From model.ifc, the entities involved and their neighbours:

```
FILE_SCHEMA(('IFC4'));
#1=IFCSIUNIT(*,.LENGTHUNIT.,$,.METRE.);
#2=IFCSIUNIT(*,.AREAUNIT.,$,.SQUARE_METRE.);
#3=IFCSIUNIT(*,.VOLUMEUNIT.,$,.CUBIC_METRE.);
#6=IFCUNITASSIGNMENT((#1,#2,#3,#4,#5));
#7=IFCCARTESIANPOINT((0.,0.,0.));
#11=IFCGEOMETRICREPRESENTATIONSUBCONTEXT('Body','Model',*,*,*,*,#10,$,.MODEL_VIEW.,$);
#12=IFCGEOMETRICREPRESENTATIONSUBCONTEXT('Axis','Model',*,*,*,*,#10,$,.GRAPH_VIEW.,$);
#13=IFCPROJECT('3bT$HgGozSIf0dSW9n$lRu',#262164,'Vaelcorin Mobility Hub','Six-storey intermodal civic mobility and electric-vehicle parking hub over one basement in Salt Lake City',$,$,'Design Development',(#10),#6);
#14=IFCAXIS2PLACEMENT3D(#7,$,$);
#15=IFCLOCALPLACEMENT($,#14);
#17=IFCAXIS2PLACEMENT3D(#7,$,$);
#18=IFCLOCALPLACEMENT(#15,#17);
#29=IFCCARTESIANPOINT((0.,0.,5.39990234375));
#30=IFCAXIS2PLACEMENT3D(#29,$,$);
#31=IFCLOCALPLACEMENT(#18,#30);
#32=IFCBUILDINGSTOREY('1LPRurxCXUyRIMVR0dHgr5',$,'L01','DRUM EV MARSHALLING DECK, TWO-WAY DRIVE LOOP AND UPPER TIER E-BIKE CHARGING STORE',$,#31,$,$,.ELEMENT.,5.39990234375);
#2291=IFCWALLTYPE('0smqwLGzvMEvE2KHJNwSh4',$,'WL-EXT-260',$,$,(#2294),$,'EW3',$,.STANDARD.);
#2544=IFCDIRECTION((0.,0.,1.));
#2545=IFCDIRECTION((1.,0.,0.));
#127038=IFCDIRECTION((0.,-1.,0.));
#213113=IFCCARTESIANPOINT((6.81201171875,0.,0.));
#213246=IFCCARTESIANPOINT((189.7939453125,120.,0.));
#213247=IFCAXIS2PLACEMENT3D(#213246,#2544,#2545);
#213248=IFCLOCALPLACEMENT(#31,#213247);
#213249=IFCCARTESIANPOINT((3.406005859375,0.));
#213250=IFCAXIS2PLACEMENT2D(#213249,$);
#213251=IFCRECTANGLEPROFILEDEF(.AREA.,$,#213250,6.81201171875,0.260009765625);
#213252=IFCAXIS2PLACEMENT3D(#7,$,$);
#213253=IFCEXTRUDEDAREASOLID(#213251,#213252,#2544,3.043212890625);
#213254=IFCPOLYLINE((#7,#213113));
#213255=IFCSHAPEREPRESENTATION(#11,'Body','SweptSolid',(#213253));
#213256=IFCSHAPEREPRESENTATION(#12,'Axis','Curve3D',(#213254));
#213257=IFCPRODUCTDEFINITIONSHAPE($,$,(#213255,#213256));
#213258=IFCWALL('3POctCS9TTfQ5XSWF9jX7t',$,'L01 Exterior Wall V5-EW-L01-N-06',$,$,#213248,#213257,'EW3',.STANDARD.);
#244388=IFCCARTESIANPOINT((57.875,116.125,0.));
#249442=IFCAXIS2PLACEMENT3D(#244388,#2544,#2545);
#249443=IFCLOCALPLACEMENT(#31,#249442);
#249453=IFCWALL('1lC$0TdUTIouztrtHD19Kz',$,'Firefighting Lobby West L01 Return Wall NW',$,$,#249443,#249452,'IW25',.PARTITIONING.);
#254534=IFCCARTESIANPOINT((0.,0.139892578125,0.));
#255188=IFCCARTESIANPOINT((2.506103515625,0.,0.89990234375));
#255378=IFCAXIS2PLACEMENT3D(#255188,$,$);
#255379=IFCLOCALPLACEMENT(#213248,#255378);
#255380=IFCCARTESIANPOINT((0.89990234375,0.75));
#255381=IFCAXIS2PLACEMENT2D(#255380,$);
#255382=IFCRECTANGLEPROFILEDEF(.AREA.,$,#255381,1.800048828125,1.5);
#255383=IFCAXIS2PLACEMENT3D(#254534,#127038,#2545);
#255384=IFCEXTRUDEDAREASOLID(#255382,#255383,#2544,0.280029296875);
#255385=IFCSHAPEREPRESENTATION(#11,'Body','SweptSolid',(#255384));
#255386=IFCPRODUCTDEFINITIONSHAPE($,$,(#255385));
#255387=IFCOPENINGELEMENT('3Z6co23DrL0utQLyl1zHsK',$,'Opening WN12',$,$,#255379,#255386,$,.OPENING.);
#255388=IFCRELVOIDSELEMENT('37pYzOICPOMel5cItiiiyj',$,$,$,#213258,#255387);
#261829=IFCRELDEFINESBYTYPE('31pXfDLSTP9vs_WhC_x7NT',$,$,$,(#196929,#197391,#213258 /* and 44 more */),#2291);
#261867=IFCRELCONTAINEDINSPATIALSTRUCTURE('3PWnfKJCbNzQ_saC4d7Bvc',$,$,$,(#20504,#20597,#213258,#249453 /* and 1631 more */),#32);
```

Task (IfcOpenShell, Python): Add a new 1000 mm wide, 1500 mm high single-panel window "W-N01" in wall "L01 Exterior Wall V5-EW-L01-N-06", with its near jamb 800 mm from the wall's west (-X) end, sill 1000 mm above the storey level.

```python
import numpy as np
import ifcopenshell
import ifcopenshell.api.feature
import ifcopenshell.api.geometry
import ifcopenshell.api.root
import ifcopenshell.api.spatial
import ifcopenshell.geom
import ifcopenshell.util.element
import ifcopenshell.util.placement
import ifcopenshell.util.representation
import ifcopenshell.util.shape
import ifcopenshell.util.unit

model = ifcopenshell.open("model.ifc")
unit_scale = ifcopenshell.util.unit.calculate_unit_scale(model)
settings = ifcopenshell.geom.settings()


def volume(element):
    """Net volume in cubic metres, openings subtracted."""
    shape = ifcopenshell.geom.create_shape(settings, element)
    return ifcopenshell.util.shape.get_volume(shape.geometry)


wall = model.by_guid("3POctCS9TTfQ5XSWF9jX7t")
storey = ifcopenshell.util.element.get_container(wall, ifc_class="IfcBuildingStorey")
context = ifcopenshell.util.representation.get_context(model, "Model", "Body", "MODEL_VIEW")
before = volume(wall)

width, height, from_end, sill = 1, 1.5, 0.8, 1  # metres

# The wall runs along its own X axis, and the end named is its -X end.
wall_shape = ifcopenshell.geom.create_shape(settings, wall)
x, y, z = ifcopenshell.util.shape.get_vertices(wall_shape.geometry).T
start = x.min() + from_end
face, thickness = float(y.min()), float(y.max() - y.min())
wall_matrix = ifcopenshell.util.placement.get_local_placement(wall.ObjectPlacement)
level = ifcopenshell.util.placement.get_local_placement(storey.ObjectPlacement)[2, 3]


def in_wall(x, y):
    """Placement at x, y metres in the wall's axes, at sill height."""
    matrix = wall_matrix.copy()
    matrix[:, 3] = wall_matrix @ np.array([x / unit_scale, y / unit_scale, 0.0, 1.0])
    matrix[2, 3] = level + sill / unit_scale
    return matrix


# Opening: a box that overshoots both wall faces by 50 mm.
opening = ifcopenshell.api.root.create_entity(model, ifc_class="IfcOpeningElement", predefined_type="OPENING")
box = ifcopenshell.api.geometry.add_wall_representation(
    model, context=context, length=width, height=height, thickness=thickness + 0.1
)
ifcopenshell.api.geometry.assign_representation(model, product=opening, representation=box)
ifcopenshell.api.geometry.edit_object_placement(model, product=opening, matrix=in_wall(start, face - 0.05), is_si=False)
ifcopenshell.api.feature.add_feature(model, feature=opening, element=wall)

window = ifcopenshell.api.root.create_entity(model, ifc_class="IfcWindow", name="W-N01", predefined_type="WINDOW")
window.OverallWidth, window.OverallHeight = width / unit_scale, height / unit_scale
window.PartitioningType = "SINGLE_PANEL"
body = ifcopenshell.api.geometry.add_window_representation(
    model,
    context=context,
    overall_width=window.OverallWidth,
    overall_height=window.OverallHeight,
    partition_type="SINGLE_PANEL",
)
ifcopenshell.api.geometry.assign_representation(model, product=window, representation=body)
ifcopenshell.api.spatial.assign_container(model, products=[window], relating_structure=storey)
ifcopenshell.api.feature.add_filling(model, opening=opening, element=window)

# Centre the window in the wall's thickness.
ifcopenshell.api.geometry.edit_object_placement(model, product=window, matrix=in_wall(start, face), is_si=False)
window_shape = ifcopenshell.geom.create_shape(settings, window)
depth = ifcopenshell.util.shape.get_vertices(window_shape.geometry)[:, 1]
offset = face + thickness / 2 - (depth.min() + depth.max()) / 2
ifcopenshell.api.geometry.edit_object_placement(model, product=window, matrix=in_wall(start, offset), is_si=False)

after = volume(wall)

print(f"wall volume {before:.3f} -> {after:.3f} m3")

model.write("model_updated.ifc")
```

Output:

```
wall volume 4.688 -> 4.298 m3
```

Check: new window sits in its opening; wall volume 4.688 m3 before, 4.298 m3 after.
